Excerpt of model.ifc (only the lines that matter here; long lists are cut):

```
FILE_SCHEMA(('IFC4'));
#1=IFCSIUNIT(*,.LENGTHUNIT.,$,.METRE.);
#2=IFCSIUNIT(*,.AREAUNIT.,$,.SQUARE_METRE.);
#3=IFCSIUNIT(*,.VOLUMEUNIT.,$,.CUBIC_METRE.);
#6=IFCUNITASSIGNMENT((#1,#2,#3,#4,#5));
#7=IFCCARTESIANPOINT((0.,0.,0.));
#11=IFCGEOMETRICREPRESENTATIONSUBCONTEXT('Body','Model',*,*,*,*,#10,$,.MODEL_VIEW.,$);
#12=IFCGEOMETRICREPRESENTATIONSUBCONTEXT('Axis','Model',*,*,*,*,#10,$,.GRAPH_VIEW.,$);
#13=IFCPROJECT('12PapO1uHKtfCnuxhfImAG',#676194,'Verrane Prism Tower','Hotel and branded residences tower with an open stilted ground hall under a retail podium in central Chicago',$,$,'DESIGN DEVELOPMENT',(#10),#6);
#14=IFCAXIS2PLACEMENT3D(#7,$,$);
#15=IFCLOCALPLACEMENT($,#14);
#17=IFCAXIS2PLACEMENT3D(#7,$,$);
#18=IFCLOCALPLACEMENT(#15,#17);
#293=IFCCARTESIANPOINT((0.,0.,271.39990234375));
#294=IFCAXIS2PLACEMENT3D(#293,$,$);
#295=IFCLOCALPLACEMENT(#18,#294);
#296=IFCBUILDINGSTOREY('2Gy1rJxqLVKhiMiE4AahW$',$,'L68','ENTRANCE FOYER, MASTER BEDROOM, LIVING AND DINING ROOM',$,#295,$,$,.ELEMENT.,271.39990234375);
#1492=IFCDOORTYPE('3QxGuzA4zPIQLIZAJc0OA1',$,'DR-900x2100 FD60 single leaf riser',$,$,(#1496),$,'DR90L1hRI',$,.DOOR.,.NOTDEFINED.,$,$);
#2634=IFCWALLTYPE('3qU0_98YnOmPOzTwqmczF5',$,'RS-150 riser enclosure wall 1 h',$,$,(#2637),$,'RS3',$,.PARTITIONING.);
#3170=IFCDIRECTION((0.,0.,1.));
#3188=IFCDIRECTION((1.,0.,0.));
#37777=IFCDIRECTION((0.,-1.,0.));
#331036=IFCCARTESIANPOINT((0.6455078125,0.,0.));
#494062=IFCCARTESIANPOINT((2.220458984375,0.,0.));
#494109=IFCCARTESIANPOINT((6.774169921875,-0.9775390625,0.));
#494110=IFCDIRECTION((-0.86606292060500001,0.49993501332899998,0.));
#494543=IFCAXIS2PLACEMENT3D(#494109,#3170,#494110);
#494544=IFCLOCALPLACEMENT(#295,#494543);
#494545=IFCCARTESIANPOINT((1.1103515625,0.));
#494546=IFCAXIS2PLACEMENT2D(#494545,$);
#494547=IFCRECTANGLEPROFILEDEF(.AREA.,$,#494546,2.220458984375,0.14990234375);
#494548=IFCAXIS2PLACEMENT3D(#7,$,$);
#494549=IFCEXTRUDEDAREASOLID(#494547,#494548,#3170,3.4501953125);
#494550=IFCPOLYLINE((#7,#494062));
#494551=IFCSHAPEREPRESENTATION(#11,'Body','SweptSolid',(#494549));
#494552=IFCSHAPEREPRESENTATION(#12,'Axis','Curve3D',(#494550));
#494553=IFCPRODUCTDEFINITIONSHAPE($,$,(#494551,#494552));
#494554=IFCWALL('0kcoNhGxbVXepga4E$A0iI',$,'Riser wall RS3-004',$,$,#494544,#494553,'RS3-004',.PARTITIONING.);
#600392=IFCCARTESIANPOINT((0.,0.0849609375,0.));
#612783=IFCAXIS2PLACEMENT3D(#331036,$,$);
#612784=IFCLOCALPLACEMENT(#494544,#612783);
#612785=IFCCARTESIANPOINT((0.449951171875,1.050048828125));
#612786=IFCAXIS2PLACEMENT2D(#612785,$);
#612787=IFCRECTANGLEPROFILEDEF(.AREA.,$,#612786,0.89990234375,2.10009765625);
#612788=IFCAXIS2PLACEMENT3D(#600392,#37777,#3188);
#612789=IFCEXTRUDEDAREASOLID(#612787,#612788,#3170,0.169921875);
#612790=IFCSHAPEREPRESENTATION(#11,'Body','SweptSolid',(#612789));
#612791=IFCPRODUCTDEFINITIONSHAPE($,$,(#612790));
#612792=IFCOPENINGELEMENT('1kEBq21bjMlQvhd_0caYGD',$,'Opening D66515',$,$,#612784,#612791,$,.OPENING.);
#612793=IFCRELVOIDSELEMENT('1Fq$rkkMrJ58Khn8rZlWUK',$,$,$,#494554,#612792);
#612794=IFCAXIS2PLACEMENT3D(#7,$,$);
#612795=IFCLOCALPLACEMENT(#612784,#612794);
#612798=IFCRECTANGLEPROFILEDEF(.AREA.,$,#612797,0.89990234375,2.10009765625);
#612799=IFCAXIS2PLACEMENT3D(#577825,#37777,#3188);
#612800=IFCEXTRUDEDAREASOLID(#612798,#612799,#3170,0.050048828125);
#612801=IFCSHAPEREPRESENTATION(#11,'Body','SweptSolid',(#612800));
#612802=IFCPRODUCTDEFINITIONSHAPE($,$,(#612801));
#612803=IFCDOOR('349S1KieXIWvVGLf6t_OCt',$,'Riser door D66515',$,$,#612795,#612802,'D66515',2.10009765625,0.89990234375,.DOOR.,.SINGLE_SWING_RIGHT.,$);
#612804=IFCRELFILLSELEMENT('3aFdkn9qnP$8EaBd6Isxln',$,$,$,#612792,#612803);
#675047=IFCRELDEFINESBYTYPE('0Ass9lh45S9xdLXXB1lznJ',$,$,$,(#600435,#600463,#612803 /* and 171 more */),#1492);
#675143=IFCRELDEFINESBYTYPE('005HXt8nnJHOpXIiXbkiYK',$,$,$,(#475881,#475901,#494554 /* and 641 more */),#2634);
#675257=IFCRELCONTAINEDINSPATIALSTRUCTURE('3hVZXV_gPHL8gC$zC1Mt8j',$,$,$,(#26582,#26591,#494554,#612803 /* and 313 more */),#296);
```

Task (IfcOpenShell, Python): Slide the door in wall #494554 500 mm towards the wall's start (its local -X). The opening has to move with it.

```python
import ifcopenshell
import ifcopenshell.api.geometry
import ifcopenshell.util.placement
import ifcopenshell.util.unit

model = ifcopenshell.open("model.ifc")
unit_scale = ifcopenshell.util.unit.calculate_unit_scale(model)

door = model.by_guid("349S1KieXIWvVGLf6t_OCt")
opening = door.FillsVoids[0].RelatingOpeningElement
wall = opening.VoidsElements[0].RelatingBuildingElement

wall_matrix = ifcopenshell.util.placement.get_local_placement(wall.ObjectPlacement)
shift = wall_matrix[:3, 0] * -0.5 / unit_scale
before = ifcopenshell.util.placement.get_local_placement(door.ObjectPlacement)[:3, 3].copy()

# The door is placed relative to its opening, so it follows when the opening moves.
matrix = ifcopenshell.util.placement.get_local_placement(opening.ObjectPlacement)
matrix[:3, 3] += shift
ifcopenshell.api.geometry.edit_object_placement(
    model, product=opening, matrix=matrix, is_si=False, should_transform_children=True
)

after = ifcopenshell.util.placement.get_local_placement(door.ObjectPlacement)[:3, 3]
print("door moved by", (after - before).round(3) + 0.0)

model.write("model_edited.ifc")
```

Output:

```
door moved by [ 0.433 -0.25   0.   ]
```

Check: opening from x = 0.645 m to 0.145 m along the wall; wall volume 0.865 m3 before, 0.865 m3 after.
